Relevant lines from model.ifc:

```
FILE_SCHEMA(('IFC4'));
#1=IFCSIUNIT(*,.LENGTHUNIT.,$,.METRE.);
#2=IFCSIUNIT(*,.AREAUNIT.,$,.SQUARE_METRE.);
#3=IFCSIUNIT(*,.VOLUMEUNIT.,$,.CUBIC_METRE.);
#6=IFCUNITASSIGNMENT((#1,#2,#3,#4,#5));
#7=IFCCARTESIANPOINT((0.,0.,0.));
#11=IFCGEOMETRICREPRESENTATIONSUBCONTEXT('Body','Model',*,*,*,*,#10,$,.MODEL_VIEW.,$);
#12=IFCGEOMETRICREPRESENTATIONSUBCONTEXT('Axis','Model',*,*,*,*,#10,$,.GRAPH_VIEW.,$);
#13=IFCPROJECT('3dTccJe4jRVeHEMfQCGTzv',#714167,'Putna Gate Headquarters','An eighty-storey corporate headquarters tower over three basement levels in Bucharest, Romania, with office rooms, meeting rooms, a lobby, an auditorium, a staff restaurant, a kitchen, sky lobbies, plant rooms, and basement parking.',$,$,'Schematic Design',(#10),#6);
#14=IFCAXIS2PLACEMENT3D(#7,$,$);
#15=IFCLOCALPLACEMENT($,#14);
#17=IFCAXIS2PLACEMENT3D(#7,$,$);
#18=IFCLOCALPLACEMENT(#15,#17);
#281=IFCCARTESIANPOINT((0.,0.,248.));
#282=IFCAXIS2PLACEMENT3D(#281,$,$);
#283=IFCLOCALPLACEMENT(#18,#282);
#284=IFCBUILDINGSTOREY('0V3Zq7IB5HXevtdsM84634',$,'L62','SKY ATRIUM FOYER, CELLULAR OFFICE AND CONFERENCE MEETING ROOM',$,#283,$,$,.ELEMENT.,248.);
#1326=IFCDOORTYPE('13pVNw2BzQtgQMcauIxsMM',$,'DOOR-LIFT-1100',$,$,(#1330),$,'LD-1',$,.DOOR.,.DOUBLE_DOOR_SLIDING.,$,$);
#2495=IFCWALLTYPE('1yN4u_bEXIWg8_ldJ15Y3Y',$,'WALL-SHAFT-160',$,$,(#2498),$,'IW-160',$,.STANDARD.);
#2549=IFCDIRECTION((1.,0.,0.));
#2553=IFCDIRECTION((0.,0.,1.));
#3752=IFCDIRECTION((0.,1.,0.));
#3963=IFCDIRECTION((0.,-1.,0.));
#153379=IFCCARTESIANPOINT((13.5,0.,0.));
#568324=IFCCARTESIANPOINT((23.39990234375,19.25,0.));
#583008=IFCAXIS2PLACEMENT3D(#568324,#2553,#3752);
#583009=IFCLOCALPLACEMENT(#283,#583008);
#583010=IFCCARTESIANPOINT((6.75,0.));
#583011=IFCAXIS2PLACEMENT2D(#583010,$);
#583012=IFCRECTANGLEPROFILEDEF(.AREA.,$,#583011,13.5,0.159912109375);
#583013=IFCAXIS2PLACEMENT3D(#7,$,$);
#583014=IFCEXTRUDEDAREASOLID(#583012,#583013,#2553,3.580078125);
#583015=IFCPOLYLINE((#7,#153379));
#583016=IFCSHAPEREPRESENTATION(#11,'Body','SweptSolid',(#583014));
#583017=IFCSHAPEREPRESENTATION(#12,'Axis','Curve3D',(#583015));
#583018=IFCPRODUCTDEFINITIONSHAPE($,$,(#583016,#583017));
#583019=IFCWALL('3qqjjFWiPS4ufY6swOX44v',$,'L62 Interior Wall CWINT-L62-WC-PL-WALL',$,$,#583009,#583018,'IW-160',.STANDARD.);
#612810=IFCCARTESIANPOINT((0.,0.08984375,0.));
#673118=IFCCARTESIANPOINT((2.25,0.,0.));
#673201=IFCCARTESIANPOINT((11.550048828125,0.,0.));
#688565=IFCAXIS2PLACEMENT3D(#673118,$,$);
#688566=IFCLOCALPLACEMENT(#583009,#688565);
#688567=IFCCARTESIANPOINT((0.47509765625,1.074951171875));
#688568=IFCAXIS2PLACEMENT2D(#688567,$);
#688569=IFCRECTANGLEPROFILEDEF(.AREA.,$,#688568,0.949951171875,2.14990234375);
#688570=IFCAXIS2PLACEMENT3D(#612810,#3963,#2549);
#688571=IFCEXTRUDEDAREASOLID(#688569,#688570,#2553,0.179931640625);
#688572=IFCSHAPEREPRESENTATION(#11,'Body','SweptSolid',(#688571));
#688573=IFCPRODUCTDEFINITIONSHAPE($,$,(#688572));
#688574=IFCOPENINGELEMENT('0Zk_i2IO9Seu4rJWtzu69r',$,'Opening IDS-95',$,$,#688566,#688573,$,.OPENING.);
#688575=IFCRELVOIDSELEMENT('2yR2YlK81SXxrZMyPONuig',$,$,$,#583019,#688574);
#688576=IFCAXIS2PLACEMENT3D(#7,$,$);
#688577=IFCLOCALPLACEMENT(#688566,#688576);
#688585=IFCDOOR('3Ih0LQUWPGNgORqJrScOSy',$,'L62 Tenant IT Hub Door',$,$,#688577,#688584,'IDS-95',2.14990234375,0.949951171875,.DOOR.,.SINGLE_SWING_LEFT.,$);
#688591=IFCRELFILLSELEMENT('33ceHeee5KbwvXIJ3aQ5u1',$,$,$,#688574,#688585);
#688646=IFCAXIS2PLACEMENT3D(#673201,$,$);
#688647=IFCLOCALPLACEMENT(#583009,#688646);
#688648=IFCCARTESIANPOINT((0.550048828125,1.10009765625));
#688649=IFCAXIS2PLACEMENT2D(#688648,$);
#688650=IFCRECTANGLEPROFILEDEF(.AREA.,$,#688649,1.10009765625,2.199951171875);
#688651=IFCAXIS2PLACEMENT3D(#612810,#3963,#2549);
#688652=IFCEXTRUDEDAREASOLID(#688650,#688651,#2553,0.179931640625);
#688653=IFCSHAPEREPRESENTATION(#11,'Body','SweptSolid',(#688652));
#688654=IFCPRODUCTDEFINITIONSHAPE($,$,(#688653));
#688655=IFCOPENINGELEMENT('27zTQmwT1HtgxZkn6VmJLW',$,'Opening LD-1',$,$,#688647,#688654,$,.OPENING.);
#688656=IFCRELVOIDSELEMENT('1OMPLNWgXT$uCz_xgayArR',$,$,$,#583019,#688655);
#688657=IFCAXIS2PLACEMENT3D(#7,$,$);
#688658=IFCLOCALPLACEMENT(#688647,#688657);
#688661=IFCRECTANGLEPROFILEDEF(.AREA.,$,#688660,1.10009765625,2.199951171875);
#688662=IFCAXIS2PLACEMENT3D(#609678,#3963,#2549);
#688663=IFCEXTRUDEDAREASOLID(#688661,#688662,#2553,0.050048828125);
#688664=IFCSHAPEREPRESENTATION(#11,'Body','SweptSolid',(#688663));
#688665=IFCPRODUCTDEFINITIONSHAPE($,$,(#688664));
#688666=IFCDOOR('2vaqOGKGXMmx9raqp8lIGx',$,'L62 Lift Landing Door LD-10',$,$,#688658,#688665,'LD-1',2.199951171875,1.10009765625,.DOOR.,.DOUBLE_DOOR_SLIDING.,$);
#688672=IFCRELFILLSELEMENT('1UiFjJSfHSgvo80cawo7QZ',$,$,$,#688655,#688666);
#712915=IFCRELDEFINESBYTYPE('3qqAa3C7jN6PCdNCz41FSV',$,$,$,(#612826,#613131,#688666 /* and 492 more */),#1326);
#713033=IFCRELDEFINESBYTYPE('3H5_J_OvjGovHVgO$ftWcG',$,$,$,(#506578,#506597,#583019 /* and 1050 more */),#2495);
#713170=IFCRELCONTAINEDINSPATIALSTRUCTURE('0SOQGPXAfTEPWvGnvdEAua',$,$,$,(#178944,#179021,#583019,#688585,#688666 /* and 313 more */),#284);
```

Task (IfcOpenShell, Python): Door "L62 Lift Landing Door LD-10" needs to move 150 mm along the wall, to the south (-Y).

```python
import ifcopenshell
import ifcopenshell.api.geometry
import ifcopenshell.util.placement
import ifcopenshell.util.unit

model = ifcopenshell.open("model.ifc")
unit_scale = ifcopenshell.util.unit.calculate_unit_scale(model)

door = model.by_guid("2vaqOGKGXMmx9raqp8lIGx")
opening = door.FillsVoids[0].RelatingOpeningElement
wall = opening.VoidsElements[0].RelatingBuildingElement

wall_matrix = ifcopenshell.util.placement.get_local_placement(wall.ObjectPlacement)
shift = wall_matrix[:3, 0] * -0.15 / unit_scale
before = ifcopenshell.util.placement.get_local_placement(door.ObjectPlacement)[:3, 3].copy()

# The door is placed relative to its opening, so it follows when the opening moves.
matrix = ifcopenshell.util.placement.get_local_placement(opening.ObjectPlacement)
matrix[:3, 3] += shift
ifcopenshell.api.geometry.edit_object_placement(
    model, product=opening, matrix=matrix, is_si=False, should_transform_children=True
)

after = ifcopenshell.util.placement.get_local_placement(door.ObjectPlacement)[:3, 3]
print("door moved by", (after - before).round(3) + 0.0)

model.write("model_v2.ifc")
```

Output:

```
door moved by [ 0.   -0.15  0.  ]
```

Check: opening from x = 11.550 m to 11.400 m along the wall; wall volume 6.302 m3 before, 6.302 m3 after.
